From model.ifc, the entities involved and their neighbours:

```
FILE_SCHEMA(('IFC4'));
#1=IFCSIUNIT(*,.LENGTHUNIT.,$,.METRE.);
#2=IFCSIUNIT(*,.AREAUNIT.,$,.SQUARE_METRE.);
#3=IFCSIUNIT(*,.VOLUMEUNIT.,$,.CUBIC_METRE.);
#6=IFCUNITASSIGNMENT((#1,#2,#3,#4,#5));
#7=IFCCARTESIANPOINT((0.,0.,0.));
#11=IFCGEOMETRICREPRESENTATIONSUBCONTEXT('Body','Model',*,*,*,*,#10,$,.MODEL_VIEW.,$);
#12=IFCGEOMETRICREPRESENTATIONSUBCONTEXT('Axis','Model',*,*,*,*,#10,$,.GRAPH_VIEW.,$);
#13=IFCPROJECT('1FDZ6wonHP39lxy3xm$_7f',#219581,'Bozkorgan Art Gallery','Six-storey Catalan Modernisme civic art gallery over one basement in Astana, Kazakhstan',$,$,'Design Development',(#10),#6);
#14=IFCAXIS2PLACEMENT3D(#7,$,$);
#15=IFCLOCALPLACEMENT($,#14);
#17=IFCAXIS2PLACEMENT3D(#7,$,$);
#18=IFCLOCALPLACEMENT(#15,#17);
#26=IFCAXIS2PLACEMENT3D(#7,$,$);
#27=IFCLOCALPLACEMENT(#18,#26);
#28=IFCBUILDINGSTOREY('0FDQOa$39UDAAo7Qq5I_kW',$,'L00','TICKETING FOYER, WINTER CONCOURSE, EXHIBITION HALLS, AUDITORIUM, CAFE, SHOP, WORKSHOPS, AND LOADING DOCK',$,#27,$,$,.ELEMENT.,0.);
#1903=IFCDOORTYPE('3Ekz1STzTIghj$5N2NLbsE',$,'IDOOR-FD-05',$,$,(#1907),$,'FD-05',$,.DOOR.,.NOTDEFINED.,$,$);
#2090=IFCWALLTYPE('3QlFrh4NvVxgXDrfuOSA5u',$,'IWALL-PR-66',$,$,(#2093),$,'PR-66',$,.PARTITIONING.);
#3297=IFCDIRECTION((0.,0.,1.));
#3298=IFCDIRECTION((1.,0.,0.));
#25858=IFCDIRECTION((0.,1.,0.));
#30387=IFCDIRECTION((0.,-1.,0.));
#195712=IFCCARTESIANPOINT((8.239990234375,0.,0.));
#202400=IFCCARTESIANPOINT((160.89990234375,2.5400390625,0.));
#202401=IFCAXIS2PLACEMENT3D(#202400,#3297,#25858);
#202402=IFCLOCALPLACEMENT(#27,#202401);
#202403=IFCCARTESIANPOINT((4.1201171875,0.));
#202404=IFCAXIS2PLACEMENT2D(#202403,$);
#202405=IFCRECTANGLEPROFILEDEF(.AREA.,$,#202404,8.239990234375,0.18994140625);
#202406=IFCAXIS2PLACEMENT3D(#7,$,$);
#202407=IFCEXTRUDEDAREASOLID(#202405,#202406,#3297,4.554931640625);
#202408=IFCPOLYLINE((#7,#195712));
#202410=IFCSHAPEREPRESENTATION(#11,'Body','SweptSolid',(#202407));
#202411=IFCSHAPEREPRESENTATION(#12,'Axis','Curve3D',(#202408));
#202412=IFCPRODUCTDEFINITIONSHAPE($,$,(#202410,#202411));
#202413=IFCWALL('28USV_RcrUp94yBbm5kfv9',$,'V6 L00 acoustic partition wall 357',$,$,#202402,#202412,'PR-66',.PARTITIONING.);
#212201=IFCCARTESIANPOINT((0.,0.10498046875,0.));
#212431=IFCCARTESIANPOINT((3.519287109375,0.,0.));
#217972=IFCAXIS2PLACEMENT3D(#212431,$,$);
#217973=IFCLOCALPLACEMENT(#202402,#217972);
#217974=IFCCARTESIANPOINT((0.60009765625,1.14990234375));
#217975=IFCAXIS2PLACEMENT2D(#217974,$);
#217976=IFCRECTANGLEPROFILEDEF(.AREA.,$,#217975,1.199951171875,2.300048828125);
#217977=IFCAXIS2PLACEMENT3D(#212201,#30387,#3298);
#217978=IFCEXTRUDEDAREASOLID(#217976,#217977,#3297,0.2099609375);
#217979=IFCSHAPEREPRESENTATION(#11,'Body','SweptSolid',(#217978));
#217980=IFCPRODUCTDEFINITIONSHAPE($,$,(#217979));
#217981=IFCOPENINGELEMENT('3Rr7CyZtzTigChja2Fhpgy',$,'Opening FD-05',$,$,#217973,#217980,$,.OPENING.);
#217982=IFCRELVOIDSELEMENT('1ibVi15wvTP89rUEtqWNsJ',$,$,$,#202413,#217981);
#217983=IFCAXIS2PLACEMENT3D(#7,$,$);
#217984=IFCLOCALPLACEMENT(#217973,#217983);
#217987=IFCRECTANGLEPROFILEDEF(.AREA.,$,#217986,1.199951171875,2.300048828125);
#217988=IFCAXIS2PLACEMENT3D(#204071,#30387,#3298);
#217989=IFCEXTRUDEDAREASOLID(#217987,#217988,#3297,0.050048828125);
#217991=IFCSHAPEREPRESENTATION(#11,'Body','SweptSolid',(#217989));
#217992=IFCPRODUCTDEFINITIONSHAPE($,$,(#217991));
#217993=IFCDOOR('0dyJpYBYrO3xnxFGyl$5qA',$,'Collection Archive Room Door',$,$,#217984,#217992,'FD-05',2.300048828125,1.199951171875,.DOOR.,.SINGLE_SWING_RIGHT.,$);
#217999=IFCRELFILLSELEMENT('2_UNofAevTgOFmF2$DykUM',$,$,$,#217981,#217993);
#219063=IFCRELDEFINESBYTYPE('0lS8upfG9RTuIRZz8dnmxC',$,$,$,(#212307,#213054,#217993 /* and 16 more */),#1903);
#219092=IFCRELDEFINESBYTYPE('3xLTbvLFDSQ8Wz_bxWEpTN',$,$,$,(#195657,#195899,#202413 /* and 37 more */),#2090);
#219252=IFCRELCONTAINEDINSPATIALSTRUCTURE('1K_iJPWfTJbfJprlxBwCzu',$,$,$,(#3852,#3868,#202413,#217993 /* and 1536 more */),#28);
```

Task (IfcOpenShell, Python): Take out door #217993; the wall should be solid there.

```python
import ifcopenshell
import ifcopenshell.api.feature
import ifcopenshell.api.root
import ifcopenshell.geom
import ifcopenshell.util.shape

model = ifcopenshell.open("model.ifc")
settings = ifcopenshell.geom.settings()


def volume(element):
    """Net volume in cubic metres, openings subtracted."""
    shape = ifcopenshell.geom.create_shape(settings, element)
    return ifcopenshell.util.shape.get_volume(shape.geometry)


door = model.by_id(217993)
opening = door.FillsVoids[0].RelatingOpeningElement
wall = opening.VoidsElements[0].RelatingBuildingElement
before = volume(wall)

ifcopenshell.api.root.remove_product(model, product=door)
ifcopenshell.api.feature.remove_feature(model, feature=opening)

after = volume(wall)

print(f"wall volume {before:.3f} -> {after:.3f} m3")

model.write("model_rev.ifc")
```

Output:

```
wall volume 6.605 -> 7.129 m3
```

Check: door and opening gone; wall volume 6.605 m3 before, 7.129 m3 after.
